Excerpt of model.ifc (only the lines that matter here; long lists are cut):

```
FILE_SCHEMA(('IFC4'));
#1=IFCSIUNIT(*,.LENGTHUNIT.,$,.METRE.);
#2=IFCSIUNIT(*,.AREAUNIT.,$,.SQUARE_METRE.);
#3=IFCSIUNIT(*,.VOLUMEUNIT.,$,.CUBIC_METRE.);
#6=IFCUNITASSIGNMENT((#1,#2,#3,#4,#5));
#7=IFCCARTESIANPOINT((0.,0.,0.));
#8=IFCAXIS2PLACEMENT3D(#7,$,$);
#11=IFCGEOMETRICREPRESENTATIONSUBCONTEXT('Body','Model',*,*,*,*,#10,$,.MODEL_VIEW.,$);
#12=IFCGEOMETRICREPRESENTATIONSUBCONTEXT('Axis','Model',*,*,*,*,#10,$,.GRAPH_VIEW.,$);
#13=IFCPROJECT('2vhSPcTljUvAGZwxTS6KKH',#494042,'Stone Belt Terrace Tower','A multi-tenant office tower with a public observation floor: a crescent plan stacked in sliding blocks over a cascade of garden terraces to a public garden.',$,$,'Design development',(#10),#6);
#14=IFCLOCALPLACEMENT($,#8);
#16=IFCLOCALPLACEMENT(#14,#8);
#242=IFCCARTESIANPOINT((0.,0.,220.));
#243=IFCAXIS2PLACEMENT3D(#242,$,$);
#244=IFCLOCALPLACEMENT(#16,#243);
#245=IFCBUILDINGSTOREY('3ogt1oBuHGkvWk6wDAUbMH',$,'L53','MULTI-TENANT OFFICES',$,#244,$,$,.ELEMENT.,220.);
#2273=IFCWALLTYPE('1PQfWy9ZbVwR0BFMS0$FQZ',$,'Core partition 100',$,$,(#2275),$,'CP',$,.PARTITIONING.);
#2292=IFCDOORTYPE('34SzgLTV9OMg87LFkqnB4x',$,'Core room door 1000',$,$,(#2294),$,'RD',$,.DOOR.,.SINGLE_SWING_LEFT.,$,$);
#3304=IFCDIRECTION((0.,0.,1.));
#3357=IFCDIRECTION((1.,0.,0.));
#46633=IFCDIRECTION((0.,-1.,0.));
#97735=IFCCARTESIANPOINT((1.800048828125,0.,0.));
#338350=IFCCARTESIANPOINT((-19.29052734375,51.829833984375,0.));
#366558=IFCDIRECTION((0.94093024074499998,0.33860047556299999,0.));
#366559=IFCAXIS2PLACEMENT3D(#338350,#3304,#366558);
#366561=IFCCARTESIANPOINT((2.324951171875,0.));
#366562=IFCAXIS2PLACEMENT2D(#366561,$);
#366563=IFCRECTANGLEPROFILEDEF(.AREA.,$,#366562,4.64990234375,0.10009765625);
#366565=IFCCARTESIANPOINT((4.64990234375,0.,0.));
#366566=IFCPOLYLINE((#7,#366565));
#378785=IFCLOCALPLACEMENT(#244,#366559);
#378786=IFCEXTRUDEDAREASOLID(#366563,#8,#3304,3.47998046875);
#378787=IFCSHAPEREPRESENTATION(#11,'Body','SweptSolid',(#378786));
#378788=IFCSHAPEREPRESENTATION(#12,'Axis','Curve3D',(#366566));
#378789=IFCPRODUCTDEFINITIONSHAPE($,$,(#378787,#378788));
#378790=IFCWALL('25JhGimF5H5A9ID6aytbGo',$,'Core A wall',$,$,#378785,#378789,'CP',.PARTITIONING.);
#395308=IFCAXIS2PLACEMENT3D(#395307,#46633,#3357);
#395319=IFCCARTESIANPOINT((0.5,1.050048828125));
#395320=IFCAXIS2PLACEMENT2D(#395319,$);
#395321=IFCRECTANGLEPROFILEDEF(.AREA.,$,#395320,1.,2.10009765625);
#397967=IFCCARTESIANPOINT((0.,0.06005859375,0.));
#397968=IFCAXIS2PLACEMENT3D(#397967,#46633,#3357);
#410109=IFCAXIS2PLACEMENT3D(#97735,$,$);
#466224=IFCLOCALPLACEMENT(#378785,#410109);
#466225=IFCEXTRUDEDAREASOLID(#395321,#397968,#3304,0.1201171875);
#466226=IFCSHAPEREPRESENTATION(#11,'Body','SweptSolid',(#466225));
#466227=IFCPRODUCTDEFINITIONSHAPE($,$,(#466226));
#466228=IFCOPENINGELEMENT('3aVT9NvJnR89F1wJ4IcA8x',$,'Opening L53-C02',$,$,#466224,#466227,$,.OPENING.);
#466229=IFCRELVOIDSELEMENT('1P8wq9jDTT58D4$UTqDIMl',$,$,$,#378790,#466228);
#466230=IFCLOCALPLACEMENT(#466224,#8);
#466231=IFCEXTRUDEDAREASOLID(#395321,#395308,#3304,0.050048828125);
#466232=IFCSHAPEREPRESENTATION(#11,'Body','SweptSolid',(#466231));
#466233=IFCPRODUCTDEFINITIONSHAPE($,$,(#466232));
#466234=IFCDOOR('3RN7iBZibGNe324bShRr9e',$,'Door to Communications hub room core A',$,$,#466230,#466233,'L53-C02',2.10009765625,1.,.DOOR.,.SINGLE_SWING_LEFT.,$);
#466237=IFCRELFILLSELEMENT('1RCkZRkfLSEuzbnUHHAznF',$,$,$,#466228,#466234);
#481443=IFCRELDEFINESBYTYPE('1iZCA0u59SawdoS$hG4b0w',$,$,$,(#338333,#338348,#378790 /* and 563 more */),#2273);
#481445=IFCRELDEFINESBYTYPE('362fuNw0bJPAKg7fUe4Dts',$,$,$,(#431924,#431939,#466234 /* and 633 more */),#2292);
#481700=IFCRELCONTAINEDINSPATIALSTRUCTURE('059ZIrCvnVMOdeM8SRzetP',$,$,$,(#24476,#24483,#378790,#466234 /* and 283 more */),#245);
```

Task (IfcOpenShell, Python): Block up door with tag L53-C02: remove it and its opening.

```python
import ifcopenshell
import ifcopenshell.api.feature
import ifcopenshell.api.root
import ifcopenshell.geom
import ifcopenshell.util.shape

model = ifcopenshell.open("model.ifc")
settings = ifcopenshell.geom.settings()


def volume(element):
    """Net volume in cubic metres, openings subtracted."""
    shape = ifcopenshell.geom.create_shape(settings, element)
    return ifcopenshell.util.shape.get_volume(shape.geometry)


door = model.by_guid("3RN7iBZibGNe324bShRr9e")
opening = door.FillsVoids[0].RelatingOpeningElement
wall = opening.VoidsElements[0].RelatingBuildingElement
before = volume(wall)

ifcopenshell.api.root.remove_product(model, product=door)
ifcopenshell.api.feature.remove_feature(model, feature=opening)

after = volume(wall)

print(f"wall volume {before:.3f} -> {after:.3f} m3")

model.write("model_updated.ifc")
```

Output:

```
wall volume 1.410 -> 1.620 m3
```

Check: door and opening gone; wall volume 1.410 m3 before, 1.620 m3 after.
